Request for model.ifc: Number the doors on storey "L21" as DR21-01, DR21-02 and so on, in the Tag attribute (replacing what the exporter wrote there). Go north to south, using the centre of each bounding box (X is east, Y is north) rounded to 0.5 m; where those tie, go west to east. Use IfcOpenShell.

First a look at what the model holds.

```python
import ifcopenshell
import ifcopenshell.util.element
import ifcopenshell.util.placement

model = ifcopenshell.open("model.ifc")
print(model.schema)
storey = next(s for s in model.by_type("IfcBuildingStorey") if s.Name == "L21")
doors = [e for e in ifcopenshell.util.element.get_decomposition(storey) if e.is_a("IfcDoor")]
for e in sorted(doors, key=lambda e: e.id()):
    origin = ifcopenshell.util.placement.get_local_placement(e.ObjectPlacement)[:3, 3]
    print(e.id(), e.Tag, e.Name, origin.round(2) + 0.0, sep=" | ")
```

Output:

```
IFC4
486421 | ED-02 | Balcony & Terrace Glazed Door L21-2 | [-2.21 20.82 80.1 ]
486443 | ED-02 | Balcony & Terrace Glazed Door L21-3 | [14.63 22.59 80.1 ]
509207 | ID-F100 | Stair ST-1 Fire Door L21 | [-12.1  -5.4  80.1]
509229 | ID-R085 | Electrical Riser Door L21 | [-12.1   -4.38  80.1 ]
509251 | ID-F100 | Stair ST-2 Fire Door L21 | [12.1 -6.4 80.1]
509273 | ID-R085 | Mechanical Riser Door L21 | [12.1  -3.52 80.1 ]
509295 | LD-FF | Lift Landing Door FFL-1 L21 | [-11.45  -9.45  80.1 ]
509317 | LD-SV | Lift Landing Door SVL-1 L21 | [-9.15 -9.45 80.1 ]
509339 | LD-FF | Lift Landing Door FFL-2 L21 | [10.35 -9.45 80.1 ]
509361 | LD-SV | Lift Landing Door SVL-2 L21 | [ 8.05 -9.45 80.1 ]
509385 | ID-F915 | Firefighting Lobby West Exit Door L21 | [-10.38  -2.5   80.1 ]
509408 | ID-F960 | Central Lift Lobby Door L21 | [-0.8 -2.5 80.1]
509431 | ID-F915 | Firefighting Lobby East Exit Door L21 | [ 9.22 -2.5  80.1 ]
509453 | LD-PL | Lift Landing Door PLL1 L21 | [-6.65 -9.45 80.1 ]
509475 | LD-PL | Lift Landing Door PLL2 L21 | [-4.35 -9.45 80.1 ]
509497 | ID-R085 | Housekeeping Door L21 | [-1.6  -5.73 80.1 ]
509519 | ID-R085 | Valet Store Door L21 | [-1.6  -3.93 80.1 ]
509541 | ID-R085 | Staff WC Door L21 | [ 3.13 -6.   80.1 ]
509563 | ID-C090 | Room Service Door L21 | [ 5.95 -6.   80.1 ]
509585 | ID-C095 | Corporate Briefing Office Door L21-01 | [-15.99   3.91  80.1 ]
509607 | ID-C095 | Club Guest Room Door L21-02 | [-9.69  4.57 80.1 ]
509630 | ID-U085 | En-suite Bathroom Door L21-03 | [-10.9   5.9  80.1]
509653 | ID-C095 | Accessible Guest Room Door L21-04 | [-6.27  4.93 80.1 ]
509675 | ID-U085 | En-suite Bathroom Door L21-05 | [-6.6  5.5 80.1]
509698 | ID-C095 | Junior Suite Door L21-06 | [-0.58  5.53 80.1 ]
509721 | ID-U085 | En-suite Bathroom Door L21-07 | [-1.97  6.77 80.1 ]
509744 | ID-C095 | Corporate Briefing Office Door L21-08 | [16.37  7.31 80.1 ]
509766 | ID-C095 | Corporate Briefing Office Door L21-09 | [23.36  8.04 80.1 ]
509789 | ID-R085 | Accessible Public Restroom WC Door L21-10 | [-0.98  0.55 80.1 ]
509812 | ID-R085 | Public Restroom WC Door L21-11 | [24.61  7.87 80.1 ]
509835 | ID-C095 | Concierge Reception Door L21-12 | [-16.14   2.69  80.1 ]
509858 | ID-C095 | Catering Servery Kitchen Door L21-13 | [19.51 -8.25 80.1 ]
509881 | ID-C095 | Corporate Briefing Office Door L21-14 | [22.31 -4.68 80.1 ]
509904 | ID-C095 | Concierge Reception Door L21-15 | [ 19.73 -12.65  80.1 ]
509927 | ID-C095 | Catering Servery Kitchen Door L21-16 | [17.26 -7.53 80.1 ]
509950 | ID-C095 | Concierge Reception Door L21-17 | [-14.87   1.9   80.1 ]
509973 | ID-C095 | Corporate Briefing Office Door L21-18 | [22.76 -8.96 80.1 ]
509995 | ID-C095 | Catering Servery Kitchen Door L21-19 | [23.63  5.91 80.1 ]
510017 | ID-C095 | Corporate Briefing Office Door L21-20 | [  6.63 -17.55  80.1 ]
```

```python
import ifcopenshell
import ifcopenshell.geom
import ifcopenshell.util.element
import ifcopenshell.util.shape

model = ifcopenshell.open("model.ifc")
settings = ifcopenshell.geom.settings()
settings.set("use-world-coords", True)


def centre(element):
    shape = ifcopenshell.geom.create_shape(settings, element)
    return ifcopenshell.util.shape.get_bbox_centroid(shape.geometry)


storey = next(s for s in model.by_type("IfcBuildingStorey") if s.Name == "L21")
doors = [e for e in ifcopenshell.util.element.get_decomposition(storey) if e.is_a("IfcDoor")]

# Insertion points can sit at a corner or the storey origin, so sort by the geometry (in metres).
centres = {e: centre(e) for e in doors}
doors.sort(key=lambda e: (-round(centres[e][1] / 0.5), centres[e][0]))

for i, e in enumerate(doors, start=1):
    number = f"DR21-{i:02d}"
    e.Tag = number
    print(e.id(), number)

model.write("model-out.ifc")
```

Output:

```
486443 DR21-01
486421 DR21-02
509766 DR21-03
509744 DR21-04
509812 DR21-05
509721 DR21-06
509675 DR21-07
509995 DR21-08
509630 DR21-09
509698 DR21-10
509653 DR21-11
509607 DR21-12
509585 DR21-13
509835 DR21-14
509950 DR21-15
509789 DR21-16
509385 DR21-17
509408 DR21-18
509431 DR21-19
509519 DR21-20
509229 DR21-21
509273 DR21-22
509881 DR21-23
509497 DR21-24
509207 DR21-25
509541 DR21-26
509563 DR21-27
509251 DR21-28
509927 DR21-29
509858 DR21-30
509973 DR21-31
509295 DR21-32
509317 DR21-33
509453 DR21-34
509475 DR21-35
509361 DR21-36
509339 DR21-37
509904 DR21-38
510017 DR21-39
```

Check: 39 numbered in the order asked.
